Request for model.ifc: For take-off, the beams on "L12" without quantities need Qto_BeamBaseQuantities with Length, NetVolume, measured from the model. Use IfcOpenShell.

First a look at what the model holds.

```python
import ifcopenshell
import ifcopenshell.util.element
import ifcopenshell.util.unit

model = ifcopenshell.open("model.ifc")
print(model.schema)
for unit_type in ("LENGTHUNIT", "AREAUNIT", "VOLUMEUNIT"):
    print(unit_type, ifcopenshell.util.unit.calculate_unit_scale(model, unit_type))
storey = next(s for s in model.by_type("IfcBuildingStorey") if s.Name == "L12")
beams = [e for e in ifcopenshell.util.element.get_decomposition(storey) if e.is_a("IfcBeam")]
for e in sorted(beams, key=lambda e: e.id()):
    print(e.id(), e.is_a(), e.Name, list(ifcopenshell.util.element.get_psets(e, qtos_only=True)), sep=" | ")
```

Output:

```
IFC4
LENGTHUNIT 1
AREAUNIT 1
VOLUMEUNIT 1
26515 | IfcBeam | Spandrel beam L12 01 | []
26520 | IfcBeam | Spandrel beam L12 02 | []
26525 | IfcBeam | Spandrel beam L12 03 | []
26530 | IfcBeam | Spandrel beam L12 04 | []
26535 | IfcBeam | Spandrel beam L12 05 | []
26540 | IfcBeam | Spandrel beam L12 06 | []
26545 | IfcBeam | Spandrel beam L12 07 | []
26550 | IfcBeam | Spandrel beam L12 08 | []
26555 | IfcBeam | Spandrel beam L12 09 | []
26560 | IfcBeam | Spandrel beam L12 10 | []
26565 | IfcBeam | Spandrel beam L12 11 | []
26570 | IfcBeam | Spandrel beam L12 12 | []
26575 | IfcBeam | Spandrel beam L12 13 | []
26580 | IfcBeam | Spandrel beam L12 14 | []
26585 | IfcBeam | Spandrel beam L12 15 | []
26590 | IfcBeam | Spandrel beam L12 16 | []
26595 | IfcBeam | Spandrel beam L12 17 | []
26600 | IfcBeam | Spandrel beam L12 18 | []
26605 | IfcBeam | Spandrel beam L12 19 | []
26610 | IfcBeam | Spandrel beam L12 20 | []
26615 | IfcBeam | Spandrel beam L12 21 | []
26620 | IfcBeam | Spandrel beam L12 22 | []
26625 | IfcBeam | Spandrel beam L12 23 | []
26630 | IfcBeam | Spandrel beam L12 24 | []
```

```python
import ifcopenshell
import ifcopenshell.api.pset
import ifcopenshell.geom
import ifcopenshell.util.element
import ifcopenshell.util.shape
import ifcopenshell.util.unit

model = ifcopenshell.open("model.ifc")
unit_scale = ifcopenshell.util.unit.calculate_unit_scale(model)
volume_scale = ifcopenshell.util.unit.calculate_unit_scale(model, "VOLUMEUNIT")
settings = ifcopenshell.geom.settings()

storey = next(s for s in model.by_type("IfcBuildingStorey") if s.Name == "L12")
beams = [e for e in ifcopenshell.util.element.get_decomposition(storey) if e.is_a("IfcBeam")]

for e in sorted(beams, key=lambda e: e.id()):
    if ifcopenshell.util.element.get_psets(e, qtos_only=True, should_inherit=False):
        continue
    # Geometry comes back in metres, in the element's own axes.
    shape = ifcopenshell.geom.create_shape(settings, e)
    values = {
        "Length": ifcopenshell.util.shape.get_max_xyz(shape.geometry) / unit_scale,
        "NetVolume": ifcopenshell.util.shape.get_volume(shape.geometry) / volume_scale,
    }
    qto = ifcopenshell.api.pset.add_qto(model, product=e, name="Qto_BeamBaseQuantities")
    ifcopenshell.api.pset.edit_qto(model, qto=qto, properties=values)
    print(e.id(), {k: round(v, 3) for k, v in values.items()})

model.write("model-out.ifc")
```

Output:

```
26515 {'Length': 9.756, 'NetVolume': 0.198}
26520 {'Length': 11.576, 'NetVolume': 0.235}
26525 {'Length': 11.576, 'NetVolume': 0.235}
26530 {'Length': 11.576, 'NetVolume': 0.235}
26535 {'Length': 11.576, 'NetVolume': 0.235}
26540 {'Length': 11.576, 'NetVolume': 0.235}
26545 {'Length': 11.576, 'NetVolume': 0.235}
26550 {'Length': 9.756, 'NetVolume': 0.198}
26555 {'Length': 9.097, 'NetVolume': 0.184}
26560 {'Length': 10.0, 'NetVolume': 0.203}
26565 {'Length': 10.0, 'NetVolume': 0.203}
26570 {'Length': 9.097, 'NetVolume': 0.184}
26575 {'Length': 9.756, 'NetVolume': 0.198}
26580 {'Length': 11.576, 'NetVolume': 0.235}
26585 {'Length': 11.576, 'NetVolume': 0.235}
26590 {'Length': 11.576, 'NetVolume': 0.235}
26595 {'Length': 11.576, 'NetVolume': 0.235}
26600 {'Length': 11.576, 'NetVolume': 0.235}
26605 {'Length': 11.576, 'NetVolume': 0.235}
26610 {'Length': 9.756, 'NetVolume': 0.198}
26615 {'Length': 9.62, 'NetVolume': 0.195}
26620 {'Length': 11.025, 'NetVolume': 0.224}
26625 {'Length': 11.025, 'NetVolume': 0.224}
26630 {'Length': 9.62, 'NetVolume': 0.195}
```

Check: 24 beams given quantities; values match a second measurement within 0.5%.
